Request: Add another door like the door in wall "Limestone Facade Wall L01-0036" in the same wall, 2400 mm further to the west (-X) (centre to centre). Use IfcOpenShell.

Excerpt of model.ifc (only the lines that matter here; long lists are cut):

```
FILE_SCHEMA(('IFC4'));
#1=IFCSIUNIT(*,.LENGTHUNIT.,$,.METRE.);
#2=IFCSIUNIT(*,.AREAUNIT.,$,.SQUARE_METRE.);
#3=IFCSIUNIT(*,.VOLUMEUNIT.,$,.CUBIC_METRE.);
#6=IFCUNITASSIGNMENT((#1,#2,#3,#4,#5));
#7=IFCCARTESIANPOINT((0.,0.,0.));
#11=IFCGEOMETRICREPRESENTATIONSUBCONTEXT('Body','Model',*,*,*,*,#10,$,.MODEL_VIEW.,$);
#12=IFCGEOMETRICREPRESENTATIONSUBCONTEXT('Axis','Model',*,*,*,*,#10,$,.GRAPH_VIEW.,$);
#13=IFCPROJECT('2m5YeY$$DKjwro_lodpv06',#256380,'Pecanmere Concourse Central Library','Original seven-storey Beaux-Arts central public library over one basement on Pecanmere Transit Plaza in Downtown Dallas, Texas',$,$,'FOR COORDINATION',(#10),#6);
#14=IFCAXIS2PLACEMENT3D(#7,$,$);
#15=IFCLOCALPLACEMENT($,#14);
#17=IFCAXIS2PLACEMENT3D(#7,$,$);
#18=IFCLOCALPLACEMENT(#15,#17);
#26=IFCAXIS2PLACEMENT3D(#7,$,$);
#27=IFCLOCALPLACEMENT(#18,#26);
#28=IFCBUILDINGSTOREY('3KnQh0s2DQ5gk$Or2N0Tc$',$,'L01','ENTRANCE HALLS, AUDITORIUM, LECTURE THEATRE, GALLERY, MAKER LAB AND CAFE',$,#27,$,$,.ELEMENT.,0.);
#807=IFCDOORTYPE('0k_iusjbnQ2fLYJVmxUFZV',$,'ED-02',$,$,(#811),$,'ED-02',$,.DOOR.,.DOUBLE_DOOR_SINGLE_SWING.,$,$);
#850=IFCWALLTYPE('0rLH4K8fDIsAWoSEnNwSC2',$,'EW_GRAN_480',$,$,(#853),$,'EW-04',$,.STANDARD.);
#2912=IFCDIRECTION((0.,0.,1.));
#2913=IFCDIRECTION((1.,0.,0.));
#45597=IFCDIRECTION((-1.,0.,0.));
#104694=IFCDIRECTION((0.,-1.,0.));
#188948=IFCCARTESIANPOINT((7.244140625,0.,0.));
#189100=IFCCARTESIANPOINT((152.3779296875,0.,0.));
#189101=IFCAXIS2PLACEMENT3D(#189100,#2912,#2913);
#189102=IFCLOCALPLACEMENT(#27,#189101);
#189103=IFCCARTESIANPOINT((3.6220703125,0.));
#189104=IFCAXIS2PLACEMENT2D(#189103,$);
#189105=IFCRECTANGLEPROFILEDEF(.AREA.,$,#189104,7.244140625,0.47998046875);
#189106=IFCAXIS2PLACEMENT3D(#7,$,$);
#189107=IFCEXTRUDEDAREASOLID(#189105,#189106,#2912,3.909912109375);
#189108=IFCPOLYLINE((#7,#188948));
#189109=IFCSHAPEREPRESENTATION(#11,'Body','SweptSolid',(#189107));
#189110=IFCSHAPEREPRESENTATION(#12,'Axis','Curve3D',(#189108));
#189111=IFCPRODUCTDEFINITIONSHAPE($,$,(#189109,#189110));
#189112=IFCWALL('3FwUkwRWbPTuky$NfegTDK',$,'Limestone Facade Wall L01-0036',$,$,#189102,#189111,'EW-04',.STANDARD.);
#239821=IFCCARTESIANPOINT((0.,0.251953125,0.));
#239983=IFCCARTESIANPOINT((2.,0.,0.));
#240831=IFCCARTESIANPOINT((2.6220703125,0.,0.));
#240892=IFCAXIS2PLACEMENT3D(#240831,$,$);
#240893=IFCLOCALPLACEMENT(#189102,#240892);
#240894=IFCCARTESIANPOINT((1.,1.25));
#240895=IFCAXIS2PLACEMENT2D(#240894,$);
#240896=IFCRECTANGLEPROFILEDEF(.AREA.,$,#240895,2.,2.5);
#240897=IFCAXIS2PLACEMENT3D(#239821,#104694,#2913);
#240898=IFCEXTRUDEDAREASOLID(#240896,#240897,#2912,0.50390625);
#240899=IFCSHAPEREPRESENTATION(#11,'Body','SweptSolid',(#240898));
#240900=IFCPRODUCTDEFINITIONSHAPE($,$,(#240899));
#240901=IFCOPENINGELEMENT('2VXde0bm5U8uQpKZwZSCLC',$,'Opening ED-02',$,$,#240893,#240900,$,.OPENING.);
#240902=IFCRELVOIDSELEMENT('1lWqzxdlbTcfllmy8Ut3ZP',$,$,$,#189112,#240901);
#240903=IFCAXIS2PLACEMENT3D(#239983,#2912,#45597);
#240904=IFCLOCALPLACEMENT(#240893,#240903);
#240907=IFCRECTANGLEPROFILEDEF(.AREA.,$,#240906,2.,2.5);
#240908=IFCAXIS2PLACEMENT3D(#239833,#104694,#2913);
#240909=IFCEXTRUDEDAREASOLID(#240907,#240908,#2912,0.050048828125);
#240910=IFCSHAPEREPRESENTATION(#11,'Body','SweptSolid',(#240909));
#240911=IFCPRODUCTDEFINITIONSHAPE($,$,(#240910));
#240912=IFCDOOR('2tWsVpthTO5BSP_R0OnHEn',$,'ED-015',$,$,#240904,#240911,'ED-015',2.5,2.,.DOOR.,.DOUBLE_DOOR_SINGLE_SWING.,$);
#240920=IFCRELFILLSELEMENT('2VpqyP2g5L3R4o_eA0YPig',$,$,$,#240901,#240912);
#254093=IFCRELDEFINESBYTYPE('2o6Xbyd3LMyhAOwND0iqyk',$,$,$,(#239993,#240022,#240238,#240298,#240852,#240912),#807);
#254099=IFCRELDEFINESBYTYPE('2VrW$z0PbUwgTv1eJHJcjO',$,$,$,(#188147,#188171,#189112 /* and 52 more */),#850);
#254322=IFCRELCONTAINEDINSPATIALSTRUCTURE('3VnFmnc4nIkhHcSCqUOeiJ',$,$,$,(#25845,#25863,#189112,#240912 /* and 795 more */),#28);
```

```python
import ifcopenshell
import ifcopenshell.api.feature
import ifcopenshell.api.geometry
import ifcopenshell.api.root
import ifcopenshell.geom
import ifcopenshell.util.element
import ifcopenshell.util.placement
import ifcopenshell.util.shape
import ifcopenshell.util.unit

model = ifcopenshell.open("model.ifc")
unit_scale = ifcopenshell.util.unit.calculate_unit_scale(model)
settings = ifcopenshell.geom.settings()


def volume(element):
    """Net volume in cubic metres, openings subtracted."""
    shape = ifcopenshell.geom.create_shape(settings, element)
    return ifcopenshell.util.shape.get_volume(shape.geometry)


door = model.by_id(240912)
opening = door.FillsVoids[0].RelatingOpeningElement
wall = opening.VoidsElements[0].RelatingBuildingElement
before = volume(wall)
shift = ifcopenshell.util.placement.get_local_placement(wall.ObjectPlacement)[:3, 0] * -2.4 / unit_scale

# copy_class copies the void relationship, type, container and properties, but no geometry.
new_opening = ifcopenshell.api.root.copy_class(model, product=opening)
new_opening.Representation = ifcopenshell.util.element.copy_deep(
    model, opening.Representation, exclude=["IfcGeometricRepresentationContext", "IfcRepresentationMap"]
)
new_door = ifcopenshell.api.root.copy_class(model, product=door)
new_door.Representation = ifcopenshell.util.element.copy_deep(
    model, door.Representation, exclude=["IfcGeometricRepresentationContext", "IfcRepresentationMap"]
)
new_door.Tag = None
ifcopenshell.api.feature.add_filling(model, opening=new_opening, element=new_door)

for old, new in ((opening, new_opening), (door, new_door)):
    matrix = ifcopenshell.util.placement.get_local_placement(old.ObjectPlacement)
    matrix[:3, 3] += shift
    ifcopenshell.api.geometry.edit_object_placement(model, product=new, matrix=matrix, is_si=False)

after = volume(wall)

print(f"wall volume {before:.3f} -> {after:.3f} m3")

model.write("model_rev.ifc")
```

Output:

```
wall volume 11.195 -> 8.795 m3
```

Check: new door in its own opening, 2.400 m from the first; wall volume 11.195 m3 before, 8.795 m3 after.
